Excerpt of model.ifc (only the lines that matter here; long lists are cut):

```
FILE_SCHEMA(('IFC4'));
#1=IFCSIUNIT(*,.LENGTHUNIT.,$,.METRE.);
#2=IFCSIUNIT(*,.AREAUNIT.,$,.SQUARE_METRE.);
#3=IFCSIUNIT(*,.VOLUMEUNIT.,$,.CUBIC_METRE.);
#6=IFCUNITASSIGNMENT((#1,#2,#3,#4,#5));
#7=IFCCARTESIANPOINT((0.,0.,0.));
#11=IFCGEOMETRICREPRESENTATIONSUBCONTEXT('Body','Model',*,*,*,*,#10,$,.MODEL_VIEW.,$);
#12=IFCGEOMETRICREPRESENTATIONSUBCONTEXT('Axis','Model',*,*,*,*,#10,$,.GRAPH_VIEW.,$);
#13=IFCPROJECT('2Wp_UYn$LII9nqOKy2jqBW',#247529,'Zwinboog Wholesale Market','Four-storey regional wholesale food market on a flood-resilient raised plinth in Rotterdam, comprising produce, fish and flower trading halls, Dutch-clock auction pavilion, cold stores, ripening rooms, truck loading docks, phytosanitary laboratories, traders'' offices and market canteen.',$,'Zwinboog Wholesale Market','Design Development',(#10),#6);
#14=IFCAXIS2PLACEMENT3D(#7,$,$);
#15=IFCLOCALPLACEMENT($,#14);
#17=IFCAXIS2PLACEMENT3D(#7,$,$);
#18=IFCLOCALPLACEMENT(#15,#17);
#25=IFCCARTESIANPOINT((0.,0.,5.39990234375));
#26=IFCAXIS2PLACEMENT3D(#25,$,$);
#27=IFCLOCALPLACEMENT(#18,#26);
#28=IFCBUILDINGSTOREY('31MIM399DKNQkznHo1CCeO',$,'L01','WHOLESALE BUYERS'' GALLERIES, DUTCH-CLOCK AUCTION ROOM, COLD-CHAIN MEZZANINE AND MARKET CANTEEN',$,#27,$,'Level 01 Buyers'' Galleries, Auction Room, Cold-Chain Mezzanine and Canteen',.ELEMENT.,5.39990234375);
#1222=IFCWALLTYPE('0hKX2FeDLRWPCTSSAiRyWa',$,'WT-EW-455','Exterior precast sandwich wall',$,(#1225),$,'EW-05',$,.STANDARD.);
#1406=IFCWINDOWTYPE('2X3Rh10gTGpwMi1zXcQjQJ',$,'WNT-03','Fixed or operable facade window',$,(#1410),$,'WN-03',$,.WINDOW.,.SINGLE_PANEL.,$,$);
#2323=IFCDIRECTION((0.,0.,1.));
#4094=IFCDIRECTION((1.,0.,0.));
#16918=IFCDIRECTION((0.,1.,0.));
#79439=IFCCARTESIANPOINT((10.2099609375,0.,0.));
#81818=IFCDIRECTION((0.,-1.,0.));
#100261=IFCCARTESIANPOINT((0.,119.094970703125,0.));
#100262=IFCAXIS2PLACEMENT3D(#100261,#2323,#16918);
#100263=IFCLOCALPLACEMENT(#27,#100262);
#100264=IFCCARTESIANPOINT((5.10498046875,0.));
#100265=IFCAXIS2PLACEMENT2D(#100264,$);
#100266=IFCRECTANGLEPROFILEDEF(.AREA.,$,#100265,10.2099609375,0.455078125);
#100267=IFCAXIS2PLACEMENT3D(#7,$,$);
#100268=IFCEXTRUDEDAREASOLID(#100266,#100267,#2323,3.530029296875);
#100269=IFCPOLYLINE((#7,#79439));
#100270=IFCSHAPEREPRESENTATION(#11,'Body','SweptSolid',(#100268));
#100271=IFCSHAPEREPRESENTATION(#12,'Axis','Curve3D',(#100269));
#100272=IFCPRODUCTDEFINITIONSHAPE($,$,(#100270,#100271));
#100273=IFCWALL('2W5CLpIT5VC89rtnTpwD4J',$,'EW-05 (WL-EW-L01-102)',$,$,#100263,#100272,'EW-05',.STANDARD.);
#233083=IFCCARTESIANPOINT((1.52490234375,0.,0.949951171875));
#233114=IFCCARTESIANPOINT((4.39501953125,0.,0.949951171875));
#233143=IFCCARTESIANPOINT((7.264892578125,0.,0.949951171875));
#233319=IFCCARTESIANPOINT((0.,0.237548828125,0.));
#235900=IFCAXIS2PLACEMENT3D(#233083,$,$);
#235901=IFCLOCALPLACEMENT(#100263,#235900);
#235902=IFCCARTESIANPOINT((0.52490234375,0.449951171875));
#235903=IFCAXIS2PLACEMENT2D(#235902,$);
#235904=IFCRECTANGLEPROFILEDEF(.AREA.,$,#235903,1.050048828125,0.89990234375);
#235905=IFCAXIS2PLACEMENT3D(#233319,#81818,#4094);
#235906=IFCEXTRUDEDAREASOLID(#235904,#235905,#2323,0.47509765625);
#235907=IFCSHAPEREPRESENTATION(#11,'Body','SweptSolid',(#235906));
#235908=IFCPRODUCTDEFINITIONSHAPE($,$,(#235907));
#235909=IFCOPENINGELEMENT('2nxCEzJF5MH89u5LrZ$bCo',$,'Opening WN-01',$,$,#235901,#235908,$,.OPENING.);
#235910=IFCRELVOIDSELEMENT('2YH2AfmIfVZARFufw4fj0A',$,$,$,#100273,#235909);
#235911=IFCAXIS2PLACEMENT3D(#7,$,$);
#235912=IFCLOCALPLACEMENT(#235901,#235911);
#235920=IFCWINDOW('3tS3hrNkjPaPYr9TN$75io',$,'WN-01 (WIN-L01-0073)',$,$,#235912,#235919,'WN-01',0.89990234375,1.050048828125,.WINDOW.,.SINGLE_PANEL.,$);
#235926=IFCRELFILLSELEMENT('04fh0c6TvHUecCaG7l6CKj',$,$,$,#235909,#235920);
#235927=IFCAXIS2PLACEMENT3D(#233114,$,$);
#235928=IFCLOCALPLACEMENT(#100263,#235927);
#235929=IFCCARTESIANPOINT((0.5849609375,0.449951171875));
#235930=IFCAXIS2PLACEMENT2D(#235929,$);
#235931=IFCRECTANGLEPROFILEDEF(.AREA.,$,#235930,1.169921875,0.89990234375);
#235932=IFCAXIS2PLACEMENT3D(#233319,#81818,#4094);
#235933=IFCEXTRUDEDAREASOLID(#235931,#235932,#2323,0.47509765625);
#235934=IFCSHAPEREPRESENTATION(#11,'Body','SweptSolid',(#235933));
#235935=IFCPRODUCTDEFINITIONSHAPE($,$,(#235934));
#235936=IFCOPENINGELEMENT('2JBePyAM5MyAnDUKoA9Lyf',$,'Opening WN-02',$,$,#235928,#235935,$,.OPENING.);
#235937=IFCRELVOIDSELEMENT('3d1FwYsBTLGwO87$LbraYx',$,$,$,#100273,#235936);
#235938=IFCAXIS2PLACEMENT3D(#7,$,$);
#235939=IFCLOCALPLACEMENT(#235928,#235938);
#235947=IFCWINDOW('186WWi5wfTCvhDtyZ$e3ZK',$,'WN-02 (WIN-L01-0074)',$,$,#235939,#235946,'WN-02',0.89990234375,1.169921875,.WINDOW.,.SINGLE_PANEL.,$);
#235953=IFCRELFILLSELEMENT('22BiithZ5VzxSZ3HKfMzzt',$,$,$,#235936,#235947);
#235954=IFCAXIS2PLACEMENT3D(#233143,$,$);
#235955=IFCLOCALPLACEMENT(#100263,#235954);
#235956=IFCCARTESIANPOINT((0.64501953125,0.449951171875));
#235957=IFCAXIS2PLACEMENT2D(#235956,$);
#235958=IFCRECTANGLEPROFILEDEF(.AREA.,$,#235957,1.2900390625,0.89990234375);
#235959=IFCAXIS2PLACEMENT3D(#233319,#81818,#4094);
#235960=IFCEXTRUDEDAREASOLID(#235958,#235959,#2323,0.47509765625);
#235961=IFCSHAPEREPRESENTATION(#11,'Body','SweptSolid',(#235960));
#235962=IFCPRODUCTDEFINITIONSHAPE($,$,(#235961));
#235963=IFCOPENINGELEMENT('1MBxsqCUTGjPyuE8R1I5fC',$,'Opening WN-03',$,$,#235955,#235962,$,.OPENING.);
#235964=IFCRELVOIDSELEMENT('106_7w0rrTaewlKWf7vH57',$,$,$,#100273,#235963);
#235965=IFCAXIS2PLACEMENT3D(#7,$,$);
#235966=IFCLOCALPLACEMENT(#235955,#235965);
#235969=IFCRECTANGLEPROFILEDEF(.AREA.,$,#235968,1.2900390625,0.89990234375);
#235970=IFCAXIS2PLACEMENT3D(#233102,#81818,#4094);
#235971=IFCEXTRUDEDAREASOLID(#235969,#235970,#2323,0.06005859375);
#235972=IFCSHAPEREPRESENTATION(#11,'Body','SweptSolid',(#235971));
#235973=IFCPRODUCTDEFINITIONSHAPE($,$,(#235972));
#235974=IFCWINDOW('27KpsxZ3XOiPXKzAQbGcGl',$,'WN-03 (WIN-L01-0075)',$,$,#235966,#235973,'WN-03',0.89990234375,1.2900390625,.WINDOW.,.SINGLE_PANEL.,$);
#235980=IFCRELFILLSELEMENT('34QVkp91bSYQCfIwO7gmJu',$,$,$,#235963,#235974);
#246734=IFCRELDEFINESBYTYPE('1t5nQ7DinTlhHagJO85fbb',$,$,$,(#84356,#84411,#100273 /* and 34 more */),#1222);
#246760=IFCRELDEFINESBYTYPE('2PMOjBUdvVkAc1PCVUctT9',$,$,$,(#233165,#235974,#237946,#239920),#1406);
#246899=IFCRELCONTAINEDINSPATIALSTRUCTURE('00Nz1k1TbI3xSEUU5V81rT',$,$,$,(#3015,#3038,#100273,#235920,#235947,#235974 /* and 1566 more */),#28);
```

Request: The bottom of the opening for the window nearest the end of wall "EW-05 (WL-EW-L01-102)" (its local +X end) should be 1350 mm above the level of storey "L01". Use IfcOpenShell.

```python
import numpy as np
import ifcopenshell
import ifcopenshell.api.geometry
import ifcopenshell.geom
import ifcopenshell.util.element
import ifcopenshell.util.placement
import ifcopenshell.util.shape
import ifcopenshell.util.unit

model = ifcopenshell.open("model.ifc")
unit_scale = ifcopenshell.util.unit.calculate_unit_scale(model)

window = model.by_guid("27KpsxZ3XOiPXKzAQbGcGl")
opening = window.FillsVoids[0].RelatingOpeningElement
storey = ifcopenshell.util.element.get_container(window, ifc_class="IfcBuildingStorey")
level = ifcopenshell.util.placement.get_local_placement(storey.ObjectPlacement)[2, 3]

# The opening's origin need not be at the sill, so measure its lowest point.
shape = ifcopenshell.geom.create_shape(ifcopenshell.geom.settings(), opening)
bottom = ifcopenshell.util.shape.get_shape_bottom_elevation(shape, shape.geometry) / unit_scale
dz = level + 1.35 / unit_scale - bottom

shift = np.array([0.0, 0.0, dz])
# The window is placed relative to its opening, so it follows when the opening moves.
matrix = ifcopenshell.util.placement.get_local_placement(opening.ObjectPlacement)
matrix[:3, 3] += shift
ifcopenshell.api.geometry.edit_object_placement(
    model, product=opening, matrix=matrix, is_si=False, should_transform_children=True
)

print(f"moved by {dz * unit_scale:+.3f} m")

model.write("model_rev.ifc")
```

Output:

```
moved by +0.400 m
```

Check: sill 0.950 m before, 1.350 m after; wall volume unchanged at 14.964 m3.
